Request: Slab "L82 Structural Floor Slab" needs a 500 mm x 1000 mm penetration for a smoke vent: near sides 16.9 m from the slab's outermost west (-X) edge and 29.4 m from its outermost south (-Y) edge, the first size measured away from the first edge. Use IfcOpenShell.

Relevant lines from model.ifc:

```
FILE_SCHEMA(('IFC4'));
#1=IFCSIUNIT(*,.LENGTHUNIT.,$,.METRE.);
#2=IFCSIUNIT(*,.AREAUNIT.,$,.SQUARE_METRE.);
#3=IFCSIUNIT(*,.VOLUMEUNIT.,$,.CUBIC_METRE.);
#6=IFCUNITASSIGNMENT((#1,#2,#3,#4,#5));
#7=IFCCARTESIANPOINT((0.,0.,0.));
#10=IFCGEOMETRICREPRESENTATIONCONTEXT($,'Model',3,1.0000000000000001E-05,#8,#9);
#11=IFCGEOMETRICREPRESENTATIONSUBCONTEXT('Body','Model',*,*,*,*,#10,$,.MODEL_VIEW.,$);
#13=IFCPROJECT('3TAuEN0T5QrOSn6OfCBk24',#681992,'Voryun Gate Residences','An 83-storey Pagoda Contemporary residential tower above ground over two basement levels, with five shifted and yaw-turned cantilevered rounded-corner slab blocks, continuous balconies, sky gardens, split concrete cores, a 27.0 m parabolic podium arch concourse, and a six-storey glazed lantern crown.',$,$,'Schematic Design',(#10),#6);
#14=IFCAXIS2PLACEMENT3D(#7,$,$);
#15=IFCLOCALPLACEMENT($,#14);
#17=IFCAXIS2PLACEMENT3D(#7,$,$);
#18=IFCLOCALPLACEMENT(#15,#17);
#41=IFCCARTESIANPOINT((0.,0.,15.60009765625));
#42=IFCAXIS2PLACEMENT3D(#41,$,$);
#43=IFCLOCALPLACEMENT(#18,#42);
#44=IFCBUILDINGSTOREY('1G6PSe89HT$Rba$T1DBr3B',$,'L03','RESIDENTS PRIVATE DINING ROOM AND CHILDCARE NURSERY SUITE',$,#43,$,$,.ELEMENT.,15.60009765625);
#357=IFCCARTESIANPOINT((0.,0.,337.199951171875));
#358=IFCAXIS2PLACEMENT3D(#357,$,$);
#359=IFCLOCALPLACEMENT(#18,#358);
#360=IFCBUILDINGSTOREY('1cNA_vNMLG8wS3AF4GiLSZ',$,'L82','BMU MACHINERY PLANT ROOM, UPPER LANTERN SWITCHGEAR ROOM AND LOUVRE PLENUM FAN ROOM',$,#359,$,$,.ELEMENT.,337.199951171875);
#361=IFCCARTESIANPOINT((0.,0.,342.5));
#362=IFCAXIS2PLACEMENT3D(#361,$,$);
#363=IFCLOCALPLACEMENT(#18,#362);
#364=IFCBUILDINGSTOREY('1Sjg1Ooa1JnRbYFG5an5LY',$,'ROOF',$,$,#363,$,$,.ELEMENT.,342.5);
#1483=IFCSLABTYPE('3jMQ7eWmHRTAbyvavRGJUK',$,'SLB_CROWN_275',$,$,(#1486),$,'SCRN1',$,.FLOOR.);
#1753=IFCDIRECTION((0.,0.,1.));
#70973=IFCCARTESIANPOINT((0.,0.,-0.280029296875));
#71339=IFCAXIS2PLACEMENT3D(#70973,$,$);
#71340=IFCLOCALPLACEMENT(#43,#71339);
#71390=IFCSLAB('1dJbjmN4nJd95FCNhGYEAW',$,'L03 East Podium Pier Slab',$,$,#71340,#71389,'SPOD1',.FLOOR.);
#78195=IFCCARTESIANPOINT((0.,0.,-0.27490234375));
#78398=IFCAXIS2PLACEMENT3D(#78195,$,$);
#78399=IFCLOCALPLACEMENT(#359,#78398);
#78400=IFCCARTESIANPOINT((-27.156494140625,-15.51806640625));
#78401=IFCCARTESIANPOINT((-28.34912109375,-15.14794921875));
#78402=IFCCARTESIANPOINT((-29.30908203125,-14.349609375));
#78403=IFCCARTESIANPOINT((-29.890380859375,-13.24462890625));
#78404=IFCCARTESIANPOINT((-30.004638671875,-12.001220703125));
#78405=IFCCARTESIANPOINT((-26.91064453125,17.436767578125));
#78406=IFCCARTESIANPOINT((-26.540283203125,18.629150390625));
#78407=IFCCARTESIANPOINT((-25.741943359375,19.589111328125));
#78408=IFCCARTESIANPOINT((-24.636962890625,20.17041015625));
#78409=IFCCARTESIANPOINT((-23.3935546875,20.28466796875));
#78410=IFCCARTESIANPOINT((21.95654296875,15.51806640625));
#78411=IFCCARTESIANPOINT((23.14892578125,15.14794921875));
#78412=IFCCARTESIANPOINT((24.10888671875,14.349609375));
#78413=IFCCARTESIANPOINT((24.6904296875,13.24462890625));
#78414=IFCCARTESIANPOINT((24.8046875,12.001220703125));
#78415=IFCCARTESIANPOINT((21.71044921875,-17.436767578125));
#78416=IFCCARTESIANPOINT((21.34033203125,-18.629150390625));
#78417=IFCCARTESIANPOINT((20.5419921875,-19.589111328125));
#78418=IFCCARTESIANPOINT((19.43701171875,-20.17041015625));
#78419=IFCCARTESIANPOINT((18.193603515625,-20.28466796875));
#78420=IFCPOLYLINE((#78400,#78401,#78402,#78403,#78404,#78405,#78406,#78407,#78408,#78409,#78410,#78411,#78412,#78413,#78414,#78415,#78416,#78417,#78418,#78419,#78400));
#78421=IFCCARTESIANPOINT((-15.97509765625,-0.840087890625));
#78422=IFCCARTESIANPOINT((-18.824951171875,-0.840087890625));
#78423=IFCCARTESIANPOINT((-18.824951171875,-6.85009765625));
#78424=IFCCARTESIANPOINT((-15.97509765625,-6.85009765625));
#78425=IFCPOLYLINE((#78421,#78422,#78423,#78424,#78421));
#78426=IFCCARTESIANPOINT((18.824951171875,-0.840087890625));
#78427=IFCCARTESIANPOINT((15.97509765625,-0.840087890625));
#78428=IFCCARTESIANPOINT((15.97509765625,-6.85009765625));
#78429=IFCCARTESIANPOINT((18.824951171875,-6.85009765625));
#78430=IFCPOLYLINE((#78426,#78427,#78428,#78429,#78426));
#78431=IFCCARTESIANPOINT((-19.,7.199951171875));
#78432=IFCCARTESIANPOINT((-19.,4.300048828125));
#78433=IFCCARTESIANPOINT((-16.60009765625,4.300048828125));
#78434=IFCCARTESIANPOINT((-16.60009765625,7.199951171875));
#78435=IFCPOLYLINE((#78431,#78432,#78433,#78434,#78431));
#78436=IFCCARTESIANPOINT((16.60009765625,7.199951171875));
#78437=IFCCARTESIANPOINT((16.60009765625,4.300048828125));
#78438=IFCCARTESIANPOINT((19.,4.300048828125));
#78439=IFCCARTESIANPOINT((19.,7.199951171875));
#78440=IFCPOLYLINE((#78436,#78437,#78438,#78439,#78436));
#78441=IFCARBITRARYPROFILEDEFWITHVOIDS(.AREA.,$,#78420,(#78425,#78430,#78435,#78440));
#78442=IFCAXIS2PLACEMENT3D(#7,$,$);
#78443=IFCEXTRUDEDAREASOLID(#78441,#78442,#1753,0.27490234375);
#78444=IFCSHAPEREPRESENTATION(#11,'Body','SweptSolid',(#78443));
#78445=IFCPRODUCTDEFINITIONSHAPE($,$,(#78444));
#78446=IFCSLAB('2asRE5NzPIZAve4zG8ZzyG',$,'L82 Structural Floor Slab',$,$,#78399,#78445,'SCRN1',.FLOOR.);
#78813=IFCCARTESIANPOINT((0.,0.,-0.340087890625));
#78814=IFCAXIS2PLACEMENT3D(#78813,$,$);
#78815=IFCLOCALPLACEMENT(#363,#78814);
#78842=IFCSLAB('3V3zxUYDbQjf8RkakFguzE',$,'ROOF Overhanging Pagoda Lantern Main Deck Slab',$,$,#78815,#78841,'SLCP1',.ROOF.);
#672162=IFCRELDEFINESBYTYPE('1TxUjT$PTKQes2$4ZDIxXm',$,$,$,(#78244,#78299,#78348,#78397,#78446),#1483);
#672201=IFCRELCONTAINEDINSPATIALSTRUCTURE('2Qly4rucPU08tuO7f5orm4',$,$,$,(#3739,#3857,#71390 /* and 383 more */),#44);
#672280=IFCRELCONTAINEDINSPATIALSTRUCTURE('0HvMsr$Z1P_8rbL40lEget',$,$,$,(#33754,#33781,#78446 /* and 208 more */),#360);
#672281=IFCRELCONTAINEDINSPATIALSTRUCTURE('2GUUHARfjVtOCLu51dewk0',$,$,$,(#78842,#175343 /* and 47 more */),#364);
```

```python
import numpy as np
import ifcopenshell
import ifcopenshell.api.feature
import ifcopenshell.api.geometry
import ifcopenshell.api.root
import ifcopenshell.geom
import ifcopenshell.util.placement
import ifcopenshell.util.representation
import ifcopenshell.util.shape
import ifcopenshell.util.unit

model = ifcopenshell.open("model.ifc")
unit_scale = ifcopenshell.util.unit.calculate_unit_scale(model)
settings = ifcopenshell.geom.settings()


def volume(element):
    """Net volume in cubic metres, openings subtracted."""
    shape = ifcopenshell.geom.create_shape(settings, element)
    return ifcopenshell.util.shape.get_volume(shape.geometry)


slab = model.by_id(78446)
before = volume(slab)

# Extent in the slab's own axes, in metres. The edges named are its -X and -Y sides.
slab_shape = ifcopenshell.geom.create_shape(settings, slab)
vertices = ifcopenshell.util.shape.get_vertices(slab_shape.geometry)
x_min, y_min, bottom = vertices.min(axis=0)
top = vertices[:, 2].max()

opening = ifcopenshell.api.root.create_entity(model, ifc_class="IfcOpeningElement", name="Smoke vent opening", predefined_type="OPENING")
context = ifcopenshell.util.representation.get_context(model, "Model", "Body", "MODEL_VIEW")
width, depth = 0.5, 1
outline = [(0.0, 0.0), (width, 0.0), (width, depth), (0.0, depth), (0.0, 0.0)]
# Overshoot both faces by 50 mm so the cut is clean.
shape = ifcopenshell.api.geometry.add_slab_representation(
    model, context=context, depth=top - bottom + 0.1, polyline=outline
)
ifcopenshell.api.geometry.assign_representation(model, product=opening, representation=shape)

matrix = ifcopenshell.util.placement.get_local_placement(slab.ObjectPlacement)
matrix[:, 3] = matrix @ np.append(np.array([x_min + 16.9, y_min + 29.4, bottom - 0.05]) / unit_scale, 1.0)
ifcopenshell.api.geometry.edit_object_placement(model, product=opening, matrix=matrix, is_si=False)
ifcopenshell.api.feature.add_feature(model, feature=opening, element=slab)

after = volume(slab)

print(f"slab volume {before:.3f} -> {after:.3f} m3")

model.write("model_rev.ifc")
```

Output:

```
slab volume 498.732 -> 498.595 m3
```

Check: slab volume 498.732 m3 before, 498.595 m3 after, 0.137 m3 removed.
